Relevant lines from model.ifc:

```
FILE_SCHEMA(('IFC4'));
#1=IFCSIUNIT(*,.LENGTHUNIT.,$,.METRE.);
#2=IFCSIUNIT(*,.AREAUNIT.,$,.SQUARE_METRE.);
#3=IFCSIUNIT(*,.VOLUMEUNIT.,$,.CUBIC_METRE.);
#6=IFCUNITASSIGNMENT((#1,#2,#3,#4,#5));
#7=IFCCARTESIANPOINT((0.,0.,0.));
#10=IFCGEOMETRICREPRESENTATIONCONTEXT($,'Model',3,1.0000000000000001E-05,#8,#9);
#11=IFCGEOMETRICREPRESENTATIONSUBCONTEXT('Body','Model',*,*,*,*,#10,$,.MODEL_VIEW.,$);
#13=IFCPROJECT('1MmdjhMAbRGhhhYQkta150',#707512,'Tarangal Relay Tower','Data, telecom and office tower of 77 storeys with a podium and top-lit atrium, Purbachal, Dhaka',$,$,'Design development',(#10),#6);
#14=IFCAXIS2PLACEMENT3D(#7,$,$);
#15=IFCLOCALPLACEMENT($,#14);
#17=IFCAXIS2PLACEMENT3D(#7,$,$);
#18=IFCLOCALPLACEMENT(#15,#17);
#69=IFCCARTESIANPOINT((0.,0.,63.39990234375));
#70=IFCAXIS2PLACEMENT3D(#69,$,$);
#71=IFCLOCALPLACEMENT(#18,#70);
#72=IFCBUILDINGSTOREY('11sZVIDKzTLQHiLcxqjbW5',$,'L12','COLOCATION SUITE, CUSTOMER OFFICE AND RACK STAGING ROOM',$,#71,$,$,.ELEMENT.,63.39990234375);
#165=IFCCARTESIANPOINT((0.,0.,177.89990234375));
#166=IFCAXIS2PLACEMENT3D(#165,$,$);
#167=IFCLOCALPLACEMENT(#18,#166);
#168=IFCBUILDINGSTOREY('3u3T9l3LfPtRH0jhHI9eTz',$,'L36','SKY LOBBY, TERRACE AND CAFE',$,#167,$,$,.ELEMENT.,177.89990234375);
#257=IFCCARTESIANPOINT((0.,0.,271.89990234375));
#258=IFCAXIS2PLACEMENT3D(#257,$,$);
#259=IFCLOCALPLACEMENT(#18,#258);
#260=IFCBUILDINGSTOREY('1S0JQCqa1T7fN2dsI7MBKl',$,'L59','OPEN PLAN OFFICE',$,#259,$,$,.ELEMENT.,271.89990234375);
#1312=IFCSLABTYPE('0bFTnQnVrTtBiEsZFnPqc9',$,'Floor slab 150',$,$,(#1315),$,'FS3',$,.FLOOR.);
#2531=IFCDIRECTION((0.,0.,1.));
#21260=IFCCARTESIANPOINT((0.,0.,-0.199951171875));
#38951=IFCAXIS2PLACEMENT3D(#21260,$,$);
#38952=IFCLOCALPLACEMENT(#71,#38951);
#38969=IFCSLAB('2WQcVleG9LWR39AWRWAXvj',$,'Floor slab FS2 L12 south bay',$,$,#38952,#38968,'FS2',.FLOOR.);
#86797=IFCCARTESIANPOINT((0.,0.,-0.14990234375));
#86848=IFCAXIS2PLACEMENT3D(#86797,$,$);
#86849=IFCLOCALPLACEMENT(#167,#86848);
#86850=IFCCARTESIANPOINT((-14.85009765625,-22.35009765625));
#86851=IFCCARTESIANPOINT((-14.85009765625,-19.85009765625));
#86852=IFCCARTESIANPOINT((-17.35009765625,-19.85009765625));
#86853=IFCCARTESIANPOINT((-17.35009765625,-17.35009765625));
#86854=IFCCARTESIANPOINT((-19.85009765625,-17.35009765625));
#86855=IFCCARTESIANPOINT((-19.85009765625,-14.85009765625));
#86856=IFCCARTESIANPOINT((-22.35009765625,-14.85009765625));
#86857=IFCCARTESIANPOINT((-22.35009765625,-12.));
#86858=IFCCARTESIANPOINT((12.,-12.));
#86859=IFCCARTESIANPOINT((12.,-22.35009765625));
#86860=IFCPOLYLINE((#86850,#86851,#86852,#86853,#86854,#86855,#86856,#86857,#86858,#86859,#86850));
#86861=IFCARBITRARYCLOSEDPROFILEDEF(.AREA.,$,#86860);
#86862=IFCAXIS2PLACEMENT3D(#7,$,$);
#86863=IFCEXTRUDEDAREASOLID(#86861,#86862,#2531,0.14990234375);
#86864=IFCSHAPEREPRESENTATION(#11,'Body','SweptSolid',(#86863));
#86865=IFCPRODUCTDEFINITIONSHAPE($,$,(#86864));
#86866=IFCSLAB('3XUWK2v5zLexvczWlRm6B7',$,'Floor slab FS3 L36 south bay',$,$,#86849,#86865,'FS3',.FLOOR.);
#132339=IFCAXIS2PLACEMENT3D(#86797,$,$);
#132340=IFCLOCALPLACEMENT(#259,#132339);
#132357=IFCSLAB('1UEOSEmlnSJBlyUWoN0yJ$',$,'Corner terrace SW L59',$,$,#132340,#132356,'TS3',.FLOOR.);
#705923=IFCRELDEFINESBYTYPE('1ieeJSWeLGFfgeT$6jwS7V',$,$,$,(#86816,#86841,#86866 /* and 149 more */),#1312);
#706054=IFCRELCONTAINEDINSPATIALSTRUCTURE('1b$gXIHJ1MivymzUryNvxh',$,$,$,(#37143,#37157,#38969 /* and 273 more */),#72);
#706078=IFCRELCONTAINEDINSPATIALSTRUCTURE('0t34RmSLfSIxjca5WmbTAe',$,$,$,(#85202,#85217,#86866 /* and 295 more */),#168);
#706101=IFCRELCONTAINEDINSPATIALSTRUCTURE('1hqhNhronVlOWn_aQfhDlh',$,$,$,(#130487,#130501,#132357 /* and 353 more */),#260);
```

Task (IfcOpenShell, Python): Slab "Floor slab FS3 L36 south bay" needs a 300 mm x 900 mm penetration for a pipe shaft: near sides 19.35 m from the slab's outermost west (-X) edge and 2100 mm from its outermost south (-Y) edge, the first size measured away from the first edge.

```python
import numpy as np
import ifcopenshell
import ifcopenshell.api.feature
import ifcopenshell.api.geometry
import ifcopenshell.api.root
import ifcopenshell.geom
import ifcopenshell.util.placement
import ifcopenshell.util.representation
import ifcopenshell.util.shape
import ifcopenshell.util.unit

model = ifcopenshell.open("model.ifc")
unit_scale = ifcopenshell.util.unit.calculate_unit_scale(model)
settings = ifcopenshell.geom.settings()


def volume(element):
    """Net volume in cubic metres, openings subtracted."""
    shape = ifcopenshell.geom.create_shape(settings, element)
    return ifcopenshell.util.shape.get_volume(shape.geometry)


slab = model.by_guid("3XUWK2v5zLexvczWlRm6B7")
before = volume(slab)

# Extent in the slab's own axes, in metres. The edges named are its -X and -Y sides.
slab_shape = ifcopenshell.geom.create_shape(settings, slab)
vertices = ifcopenshell.util.shape.get_vertices(slab_shape.geometry)
x_min, y_min, bottom = vertices.min(axis=0)
top = vertices[:, 2].max()

opening = ifcopenshell.api.root.create_entity(model, ifc_class="IfcOpeningElement", name="Pipe shaft opening", predefined_type="OPENING")
context = ifcopenshell.util.representation.get_context(model, "Model", "Body", "MODEL_VIEW")
width, depth = 0.3, 0.9
outline = [(0.0, 0.0), (width, 0.0), (width, depth), (0.0, depth), (0.0, 0.0)]
# Overshoot both faces by 50 mm so the cut is clean.
shape = ifcopenshell.api.geometry.add_slab_representation(
    model, context=context, depth=top - bottom + 0.1, polyline=outline
)
ifcopenshell.api.geometry.assign_representation(model, product=opening, representation=shape)

matrix = ifcopenshell.util.placement.get_local_placement(slab.ObjectPlacement)
matrix[:, 3] = matrix @ np.append(np.array([x_min + 19.35, y_min + 2.1, bottom - 0.05]) / unit_scale, 1.0)
ifcopenshell.api.geometry.edit_object_placement(model, product=opening, matrix=matrix, is_si=False)
ifcopenshell.api.feature.add_feature(model, feature=opening, element=slab)

after = volume(slab)

print(f"slab volume {before:.3f} -> {after:.3f} m3")

model.write("model_updated.ifc")
```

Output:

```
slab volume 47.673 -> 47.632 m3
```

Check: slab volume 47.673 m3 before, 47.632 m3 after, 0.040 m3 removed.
